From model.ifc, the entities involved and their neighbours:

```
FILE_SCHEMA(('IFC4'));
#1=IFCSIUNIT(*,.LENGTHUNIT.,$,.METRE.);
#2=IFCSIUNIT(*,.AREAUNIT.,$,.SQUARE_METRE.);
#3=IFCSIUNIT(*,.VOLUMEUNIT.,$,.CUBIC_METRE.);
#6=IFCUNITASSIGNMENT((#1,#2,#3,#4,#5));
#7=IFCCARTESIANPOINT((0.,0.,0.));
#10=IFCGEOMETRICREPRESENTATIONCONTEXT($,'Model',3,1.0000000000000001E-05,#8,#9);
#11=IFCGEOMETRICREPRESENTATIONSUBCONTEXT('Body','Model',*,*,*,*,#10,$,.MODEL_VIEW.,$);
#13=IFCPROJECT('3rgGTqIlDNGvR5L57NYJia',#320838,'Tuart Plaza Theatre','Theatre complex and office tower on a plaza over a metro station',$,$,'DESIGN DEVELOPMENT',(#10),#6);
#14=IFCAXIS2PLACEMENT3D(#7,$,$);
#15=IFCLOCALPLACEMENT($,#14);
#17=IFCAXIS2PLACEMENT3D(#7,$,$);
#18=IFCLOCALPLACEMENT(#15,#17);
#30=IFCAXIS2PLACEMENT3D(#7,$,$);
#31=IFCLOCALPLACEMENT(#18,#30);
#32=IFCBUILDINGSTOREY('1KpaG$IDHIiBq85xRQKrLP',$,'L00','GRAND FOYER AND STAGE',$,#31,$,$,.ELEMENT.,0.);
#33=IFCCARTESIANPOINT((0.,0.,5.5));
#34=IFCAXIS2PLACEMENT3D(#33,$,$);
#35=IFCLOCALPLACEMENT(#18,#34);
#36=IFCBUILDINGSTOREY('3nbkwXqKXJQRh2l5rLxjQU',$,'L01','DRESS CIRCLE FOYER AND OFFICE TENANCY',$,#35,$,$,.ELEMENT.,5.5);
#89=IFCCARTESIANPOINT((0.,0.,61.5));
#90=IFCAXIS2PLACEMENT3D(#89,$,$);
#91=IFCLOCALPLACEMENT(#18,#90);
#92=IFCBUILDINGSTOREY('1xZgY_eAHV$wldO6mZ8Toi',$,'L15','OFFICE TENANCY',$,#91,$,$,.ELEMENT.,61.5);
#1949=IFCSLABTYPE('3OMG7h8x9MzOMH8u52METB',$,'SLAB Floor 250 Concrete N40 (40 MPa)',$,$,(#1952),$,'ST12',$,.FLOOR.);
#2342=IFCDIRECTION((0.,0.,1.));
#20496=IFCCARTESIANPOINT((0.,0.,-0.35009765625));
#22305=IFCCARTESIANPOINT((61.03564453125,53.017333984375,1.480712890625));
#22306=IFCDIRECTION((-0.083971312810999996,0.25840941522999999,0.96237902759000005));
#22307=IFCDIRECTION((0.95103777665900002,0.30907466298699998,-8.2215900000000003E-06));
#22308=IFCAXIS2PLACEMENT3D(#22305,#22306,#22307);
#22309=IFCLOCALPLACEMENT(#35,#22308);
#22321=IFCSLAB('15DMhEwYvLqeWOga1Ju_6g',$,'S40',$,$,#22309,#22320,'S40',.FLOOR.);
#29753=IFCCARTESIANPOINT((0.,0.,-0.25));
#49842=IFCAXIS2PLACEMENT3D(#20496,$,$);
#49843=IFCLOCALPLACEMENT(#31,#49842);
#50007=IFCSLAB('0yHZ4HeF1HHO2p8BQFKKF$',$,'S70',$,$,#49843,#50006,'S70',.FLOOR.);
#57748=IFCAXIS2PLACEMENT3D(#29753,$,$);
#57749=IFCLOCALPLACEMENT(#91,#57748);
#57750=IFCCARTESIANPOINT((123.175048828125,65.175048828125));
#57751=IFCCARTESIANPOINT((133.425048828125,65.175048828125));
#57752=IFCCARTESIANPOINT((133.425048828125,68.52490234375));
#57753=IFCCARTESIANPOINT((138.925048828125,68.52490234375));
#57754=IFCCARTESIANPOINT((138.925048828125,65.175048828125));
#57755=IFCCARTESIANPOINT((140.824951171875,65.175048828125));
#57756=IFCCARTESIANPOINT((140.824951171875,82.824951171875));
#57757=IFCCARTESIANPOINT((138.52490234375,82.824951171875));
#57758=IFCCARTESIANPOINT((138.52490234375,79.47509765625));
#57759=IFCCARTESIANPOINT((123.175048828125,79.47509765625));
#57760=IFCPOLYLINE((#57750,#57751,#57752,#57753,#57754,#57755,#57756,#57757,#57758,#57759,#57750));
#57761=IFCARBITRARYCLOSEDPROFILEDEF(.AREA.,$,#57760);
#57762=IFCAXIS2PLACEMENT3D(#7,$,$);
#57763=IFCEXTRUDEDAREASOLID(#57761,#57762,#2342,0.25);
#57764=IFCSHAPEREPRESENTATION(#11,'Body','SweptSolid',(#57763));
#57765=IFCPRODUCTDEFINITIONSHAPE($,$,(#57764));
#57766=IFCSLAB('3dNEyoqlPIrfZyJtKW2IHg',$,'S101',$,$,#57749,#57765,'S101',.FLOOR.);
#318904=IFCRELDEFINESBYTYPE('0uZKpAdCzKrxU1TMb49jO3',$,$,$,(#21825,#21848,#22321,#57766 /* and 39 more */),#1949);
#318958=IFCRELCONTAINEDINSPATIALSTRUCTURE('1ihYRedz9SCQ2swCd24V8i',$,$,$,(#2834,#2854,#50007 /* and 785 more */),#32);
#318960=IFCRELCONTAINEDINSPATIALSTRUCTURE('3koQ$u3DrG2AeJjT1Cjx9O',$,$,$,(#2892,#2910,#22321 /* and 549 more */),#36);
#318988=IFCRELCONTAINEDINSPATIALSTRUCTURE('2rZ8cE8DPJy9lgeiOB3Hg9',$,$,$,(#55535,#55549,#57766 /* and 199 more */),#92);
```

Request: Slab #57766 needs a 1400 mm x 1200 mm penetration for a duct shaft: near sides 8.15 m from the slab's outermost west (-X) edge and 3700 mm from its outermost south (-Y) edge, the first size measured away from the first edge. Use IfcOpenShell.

```python
import numpy as np
import ifcopenshell
import ifcopenshell.api.feature
import ifcopenshell.api.geometry
import ifcopenshell.api.root
import ifcopenshell.geom
import ifcopenshell.util.placement
import ifcopenshell.util.representation
import ifcopenshell.util.shape
import ifcopenshell.util.unit

model = ifcopenshell.open("model.ifc")
unit_scale = ifcopenshell.util.unit.calculate_unit_scale(model)
settings = ifcopenshell.geom.settings()


def volume(element):
    """Net volume in cubic metres, openings subtracted."""
    shape = ifcopenshell.geom.create_shape(settings, element)
    return ifcopenshell.util.shape.get_volume(shape.geometry)


slab = model.by_guid("3dNEyoqlPIrfZyJtKW2IHg")
before = volume(slab)

# Extent in the slab's own axes, in metres. The edges named are its -X and -Y sides.
slab_shape = ifcopenshell.geom.create_shape(settings, slab)
vertices = ifcopenshell.util.shape.get_vertices(slab_shape.geometry)
x_min, y_min, bottom = vertices.min(axis=0)
top = vertices[:, 2].max()

opening = ifcopenshell.api.root.create_entity(model, ifc_class="IfcOpeningElement", name="Duct shaft opening", predefined_type="OPENING")
context = ifcopenshell.util.representation.get_context(model, "Model", "Body", "MODEL_VIEW")
width, depth = 1.4, 1.2
outline = [(0.0, 0.0), (width, 0.0), (width, depth), (0.0, depth), (0.0, 0.0)]
# Overshoot both faces by 50 mm so the cut is clean.
shape = ifcopenshell.api.geometry.add_slab_representation(
    model, context=context, depth=top - bottom + 0.1, polyline=outline
)
ifcopenshell.api.geometry.assign_representation(model, product=opening, representation=shape)

matrix = ifcopenshell.util.placement.get_local_placement(slab.ObjectPlacement)
matrix[:, 3] = matrix @ np.append(np.array([x_min + 8.15, y_min + 3.7, bottom - 0.05]) / unit_scale, 1.0)
ifcopenshell.api.geometry.edit_object_placement(model, product=opening, matrix=matrix, is_si=False)
ifcopenshell.api.feature.add_feature(model, feature=opening, element=slab)

after = volume(slab)

print(f"slab volume {before:.3f} -> {after:.3f} m3")

model.write("model_v2.ifc")
```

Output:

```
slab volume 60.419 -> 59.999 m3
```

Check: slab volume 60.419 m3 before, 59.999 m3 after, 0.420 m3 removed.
